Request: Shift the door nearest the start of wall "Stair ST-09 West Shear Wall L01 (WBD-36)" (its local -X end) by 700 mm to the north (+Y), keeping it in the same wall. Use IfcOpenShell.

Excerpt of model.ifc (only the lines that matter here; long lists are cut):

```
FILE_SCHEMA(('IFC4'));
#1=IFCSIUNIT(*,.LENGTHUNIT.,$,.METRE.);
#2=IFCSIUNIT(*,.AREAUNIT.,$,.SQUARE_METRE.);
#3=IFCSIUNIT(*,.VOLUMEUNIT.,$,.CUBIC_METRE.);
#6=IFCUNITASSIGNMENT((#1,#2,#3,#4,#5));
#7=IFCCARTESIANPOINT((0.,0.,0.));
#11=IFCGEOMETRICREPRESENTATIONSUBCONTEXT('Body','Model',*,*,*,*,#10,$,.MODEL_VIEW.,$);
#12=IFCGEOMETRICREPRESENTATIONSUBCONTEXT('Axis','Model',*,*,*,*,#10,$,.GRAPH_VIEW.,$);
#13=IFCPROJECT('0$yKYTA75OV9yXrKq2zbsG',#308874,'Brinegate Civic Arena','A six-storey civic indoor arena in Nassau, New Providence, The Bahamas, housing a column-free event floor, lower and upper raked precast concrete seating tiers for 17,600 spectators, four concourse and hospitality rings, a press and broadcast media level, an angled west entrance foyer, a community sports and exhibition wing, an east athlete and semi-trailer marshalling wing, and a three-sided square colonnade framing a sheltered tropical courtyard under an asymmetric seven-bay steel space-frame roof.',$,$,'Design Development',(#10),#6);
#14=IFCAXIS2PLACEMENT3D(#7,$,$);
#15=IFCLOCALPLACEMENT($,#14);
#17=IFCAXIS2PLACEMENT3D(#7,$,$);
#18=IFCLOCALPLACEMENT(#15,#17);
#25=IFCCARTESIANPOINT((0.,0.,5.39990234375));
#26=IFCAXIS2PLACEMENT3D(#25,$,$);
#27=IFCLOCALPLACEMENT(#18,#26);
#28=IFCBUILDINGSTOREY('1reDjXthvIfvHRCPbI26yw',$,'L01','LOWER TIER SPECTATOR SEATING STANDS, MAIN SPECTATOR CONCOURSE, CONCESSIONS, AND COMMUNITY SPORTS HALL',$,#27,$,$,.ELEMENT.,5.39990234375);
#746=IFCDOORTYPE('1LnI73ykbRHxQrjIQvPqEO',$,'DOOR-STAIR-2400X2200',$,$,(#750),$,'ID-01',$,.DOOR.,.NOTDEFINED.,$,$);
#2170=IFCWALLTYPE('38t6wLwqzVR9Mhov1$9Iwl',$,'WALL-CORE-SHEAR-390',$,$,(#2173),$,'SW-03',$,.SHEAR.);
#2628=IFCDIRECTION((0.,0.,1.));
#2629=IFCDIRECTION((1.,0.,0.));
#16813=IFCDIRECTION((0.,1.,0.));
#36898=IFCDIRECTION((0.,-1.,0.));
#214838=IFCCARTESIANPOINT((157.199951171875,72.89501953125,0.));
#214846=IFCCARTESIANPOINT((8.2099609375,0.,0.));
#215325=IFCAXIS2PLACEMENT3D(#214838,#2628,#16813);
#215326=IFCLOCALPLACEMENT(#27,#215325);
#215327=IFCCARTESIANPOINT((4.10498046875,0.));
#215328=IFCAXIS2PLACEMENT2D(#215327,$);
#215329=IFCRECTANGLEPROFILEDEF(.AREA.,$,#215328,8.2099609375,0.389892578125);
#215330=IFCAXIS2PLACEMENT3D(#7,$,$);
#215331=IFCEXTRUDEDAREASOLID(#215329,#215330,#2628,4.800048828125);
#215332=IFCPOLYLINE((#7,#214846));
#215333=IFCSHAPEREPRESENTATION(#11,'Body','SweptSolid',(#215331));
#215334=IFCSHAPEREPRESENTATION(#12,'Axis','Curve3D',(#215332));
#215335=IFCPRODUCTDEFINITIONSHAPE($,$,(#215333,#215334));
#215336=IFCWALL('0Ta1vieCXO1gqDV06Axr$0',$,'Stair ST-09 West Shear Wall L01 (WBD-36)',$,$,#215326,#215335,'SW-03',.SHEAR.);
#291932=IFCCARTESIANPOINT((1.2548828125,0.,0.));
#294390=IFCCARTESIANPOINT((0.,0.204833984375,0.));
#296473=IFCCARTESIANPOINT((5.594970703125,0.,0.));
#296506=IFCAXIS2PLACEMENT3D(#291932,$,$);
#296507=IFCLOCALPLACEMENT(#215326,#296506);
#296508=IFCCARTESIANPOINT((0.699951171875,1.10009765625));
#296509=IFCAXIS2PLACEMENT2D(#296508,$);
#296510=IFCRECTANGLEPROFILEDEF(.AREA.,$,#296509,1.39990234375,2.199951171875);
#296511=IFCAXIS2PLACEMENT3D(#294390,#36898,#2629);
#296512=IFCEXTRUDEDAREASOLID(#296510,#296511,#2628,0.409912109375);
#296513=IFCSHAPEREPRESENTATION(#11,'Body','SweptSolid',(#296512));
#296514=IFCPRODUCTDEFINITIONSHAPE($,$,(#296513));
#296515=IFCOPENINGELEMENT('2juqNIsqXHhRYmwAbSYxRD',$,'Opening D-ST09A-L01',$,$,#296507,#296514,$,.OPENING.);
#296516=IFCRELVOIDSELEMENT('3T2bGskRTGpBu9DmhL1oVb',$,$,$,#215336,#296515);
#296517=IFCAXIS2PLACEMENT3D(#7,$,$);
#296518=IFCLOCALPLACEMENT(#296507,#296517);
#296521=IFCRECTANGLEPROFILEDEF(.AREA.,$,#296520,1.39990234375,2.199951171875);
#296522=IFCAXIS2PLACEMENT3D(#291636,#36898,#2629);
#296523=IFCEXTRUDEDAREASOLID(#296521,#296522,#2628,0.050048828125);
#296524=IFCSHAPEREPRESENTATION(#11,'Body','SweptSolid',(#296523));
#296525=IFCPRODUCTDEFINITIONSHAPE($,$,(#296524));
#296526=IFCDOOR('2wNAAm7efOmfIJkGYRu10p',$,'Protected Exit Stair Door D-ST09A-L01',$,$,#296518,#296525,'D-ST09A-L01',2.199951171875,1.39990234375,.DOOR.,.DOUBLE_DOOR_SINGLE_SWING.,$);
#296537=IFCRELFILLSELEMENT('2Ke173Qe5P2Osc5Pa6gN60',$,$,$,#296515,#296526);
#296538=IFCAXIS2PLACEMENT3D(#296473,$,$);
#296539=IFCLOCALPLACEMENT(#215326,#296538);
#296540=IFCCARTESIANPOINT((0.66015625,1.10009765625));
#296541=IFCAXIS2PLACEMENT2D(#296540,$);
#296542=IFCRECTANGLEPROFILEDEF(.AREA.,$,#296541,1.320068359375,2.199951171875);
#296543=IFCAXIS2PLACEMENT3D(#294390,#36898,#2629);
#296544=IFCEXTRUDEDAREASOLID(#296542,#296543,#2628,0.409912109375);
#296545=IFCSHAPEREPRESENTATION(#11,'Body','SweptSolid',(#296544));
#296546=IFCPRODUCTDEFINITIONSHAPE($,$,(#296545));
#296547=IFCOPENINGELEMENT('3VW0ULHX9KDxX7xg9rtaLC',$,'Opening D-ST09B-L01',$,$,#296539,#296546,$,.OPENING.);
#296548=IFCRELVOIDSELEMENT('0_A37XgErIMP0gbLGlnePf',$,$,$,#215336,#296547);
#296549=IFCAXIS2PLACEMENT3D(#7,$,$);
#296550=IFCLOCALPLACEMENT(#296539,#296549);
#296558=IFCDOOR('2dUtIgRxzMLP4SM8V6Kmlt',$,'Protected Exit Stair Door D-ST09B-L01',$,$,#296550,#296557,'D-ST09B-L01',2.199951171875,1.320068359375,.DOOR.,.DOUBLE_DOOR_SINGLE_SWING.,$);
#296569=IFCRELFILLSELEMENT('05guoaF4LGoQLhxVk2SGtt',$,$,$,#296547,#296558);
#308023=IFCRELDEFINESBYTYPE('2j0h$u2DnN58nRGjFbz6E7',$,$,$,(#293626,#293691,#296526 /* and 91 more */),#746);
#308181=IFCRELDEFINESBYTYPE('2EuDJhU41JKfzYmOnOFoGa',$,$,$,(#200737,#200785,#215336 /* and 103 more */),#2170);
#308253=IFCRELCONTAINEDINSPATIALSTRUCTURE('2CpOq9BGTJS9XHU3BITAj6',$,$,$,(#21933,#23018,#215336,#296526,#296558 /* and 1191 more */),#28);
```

```python
import ifcopenshell
import ifcopenshell.api.geometry
import ifcopenshell.util.placement
import ifcopenshell.util.unit

model = ifcopenshell.open("model.ifc")
unit_scale = ifcopenshell.util.unit.calculate_unit_scale(model)

door = model.by_guid("2wNAAm7efOmfIJkGYRu10p")
opening = door.FillsVoids[0].RelatingOpeningElement
wall = opening.VoidsElements[0].RelatingBuildingElement

wall_matrix = ifcopenshell.util.placement.get_local_placement(wall.ObjectPlacement)
shift = wall_matrix[:3, 0] * 0.7 / unit_scale
before = ifcopenshell.util.placement.get_local_placement(door.ObjectPlacement)[:3, 3].copy()

# The door is placed relative to its opening, so it follows when the opening moves.
matrix = ifcopenshell.util.placement.get_local_placement(opening.ObjectPlacement)
matrix[:3, 3] += shift
ifcopenshell.api.geometry.edit_object_placement(
    model, product=opening, matrix=matrix, is_si=False, should_transform_children=True
)

after = ifcopenshell.util.placement.get_local_placement(door.ObjectPlacement)[:3, 3]
print("door moved by", (after - before).round(3) + 0.0)

model.write("model_edited.ifc")
```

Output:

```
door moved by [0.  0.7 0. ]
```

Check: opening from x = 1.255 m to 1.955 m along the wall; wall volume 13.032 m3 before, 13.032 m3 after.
